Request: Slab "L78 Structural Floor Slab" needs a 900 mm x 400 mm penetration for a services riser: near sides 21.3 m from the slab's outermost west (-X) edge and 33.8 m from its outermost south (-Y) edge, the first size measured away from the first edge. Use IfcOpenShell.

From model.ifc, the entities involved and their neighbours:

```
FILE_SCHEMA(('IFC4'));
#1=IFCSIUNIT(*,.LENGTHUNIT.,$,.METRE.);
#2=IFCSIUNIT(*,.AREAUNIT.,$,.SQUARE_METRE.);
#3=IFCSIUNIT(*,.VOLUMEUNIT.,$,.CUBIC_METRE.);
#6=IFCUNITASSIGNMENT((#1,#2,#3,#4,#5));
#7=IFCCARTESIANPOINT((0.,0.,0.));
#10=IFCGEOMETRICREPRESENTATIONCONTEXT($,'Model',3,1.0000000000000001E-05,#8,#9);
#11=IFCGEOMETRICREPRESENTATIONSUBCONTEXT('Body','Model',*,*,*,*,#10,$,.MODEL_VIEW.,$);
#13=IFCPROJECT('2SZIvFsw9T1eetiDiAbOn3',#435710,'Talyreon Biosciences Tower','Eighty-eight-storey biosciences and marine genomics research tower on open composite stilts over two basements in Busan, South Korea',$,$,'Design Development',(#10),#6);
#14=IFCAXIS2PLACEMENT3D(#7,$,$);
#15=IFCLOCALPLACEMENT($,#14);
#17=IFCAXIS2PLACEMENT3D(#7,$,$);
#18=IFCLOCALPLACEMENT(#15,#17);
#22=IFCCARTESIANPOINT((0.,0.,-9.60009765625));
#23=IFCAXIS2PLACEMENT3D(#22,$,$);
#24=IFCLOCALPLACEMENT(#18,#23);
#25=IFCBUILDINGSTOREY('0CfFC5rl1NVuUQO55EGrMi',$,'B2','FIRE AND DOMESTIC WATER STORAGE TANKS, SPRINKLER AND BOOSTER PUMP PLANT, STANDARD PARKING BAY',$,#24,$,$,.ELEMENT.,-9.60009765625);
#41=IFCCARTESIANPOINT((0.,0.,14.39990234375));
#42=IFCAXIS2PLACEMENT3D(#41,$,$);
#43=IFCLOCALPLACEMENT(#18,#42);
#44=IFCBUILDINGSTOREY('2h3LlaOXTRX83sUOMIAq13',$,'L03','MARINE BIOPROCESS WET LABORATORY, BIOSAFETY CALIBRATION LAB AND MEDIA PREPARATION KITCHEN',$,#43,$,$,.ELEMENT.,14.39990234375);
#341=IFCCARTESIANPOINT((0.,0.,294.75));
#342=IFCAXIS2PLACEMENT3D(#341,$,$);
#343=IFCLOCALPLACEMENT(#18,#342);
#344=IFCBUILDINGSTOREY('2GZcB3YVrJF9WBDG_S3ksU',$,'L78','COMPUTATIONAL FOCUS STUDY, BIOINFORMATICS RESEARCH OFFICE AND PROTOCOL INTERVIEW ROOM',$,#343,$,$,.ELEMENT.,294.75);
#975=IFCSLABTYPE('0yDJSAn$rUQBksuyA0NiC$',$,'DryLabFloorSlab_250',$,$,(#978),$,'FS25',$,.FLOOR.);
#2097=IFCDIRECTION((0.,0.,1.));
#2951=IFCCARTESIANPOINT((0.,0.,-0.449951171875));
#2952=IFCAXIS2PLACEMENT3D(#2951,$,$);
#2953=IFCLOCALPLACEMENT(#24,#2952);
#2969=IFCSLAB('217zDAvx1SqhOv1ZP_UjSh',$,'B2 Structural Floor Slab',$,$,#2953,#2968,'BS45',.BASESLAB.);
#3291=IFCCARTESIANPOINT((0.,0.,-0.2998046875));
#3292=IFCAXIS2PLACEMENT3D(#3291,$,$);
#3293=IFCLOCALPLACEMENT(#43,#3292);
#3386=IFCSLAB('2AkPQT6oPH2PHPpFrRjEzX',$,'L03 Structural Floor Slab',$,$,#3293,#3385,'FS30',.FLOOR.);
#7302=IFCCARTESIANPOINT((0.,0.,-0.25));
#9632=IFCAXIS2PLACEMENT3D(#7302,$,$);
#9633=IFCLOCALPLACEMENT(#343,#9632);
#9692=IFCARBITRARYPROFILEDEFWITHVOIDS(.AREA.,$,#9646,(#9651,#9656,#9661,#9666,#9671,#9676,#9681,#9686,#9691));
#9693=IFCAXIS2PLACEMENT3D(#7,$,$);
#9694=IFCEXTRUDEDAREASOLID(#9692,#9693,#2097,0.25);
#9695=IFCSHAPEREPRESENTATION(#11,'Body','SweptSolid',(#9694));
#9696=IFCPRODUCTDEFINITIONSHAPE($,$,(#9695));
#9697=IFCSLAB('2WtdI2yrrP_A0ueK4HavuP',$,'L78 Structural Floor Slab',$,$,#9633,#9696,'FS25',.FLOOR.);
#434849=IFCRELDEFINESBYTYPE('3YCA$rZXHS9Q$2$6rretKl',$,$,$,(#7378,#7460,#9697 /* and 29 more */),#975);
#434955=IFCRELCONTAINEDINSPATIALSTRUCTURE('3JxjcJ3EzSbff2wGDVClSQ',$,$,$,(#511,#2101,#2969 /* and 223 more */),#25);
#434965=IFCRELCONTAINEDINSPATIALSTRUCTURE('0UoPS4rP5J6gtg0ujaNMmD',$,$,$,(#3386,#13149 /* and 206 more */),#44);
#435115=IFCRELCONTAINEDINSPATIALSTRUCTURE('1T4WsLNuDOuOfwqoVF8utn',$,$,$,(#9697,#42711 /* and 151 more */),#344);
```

```python
import numpy as np
import ifcopenshell
import ifcopenshell.api.feature
import ifcopenshell.api.geometry
import ifcopenshell.api.root
import ifcopenshell.geom
import ifcopenshell.util.placement
import ifcopenshell.util.representation
import ifcopenshell.util.shape
import ifcopenshell.util.unit

model = ifcopenshell.open("model.ifc")
unit_scale = ifcopenshell.util.unit.calculate_unit_scale(model)
settings = ifcopenshell.geom.settings()


def volume(element):
    """Net volume in cubic metres, openings subtracted."""
    shape = ifcopenshell.geom.create_shape(settings, element)
    return ifcopenshell.util.shape.get_volume(shape.geometry)


slab = model.by_guid("2WtdI2yrrP_A0ueK4HavuP")
before = volume(slab)

# Extent in the slab's own axes, in metres. The edges named are its -X and -Y sides.
slab_shape = ifcopenshell.geom.create_shape(settings, slab)
vertices = ifcopenshell.util.shape.get_vertices(slab_shape.geometry)
x_min, y_min, bottom = vertices.min(axis=0)
top = vertices[:, 2].max()

opening = ifcopenshell.api.root.create_entity(model, ifc_class="IfcOpeningElement", name="Services riser opening", predefined_type="OPENING")
context = ifcopenshell.util.representation.get_context(model, "Model", "Body", "MODEL_VIEW")
width, depth = 0.9, 0.4
outline = [(0.0, 0.0), (width, 0.0), (width, depth), (0.0, depth), (0.0, 0.0)]
# Overshoot both faces by 50 mm so the cut is clean.
shape = ifcopenshell.api.geometry.add_slab_representation(
    model, context=context, depth=top - bottom + 0.1, polyline=outline
)
ifcopenshell.api.geometry.assign_representation(model, product=opening, representation=shape)

matrix = ifcopenshell.util.placement.get_local_placement(slab.ObjectPlacement)
matrix[:, 3] = matrix @ np.append(np.array([x_min + 21.3, y_min + 33.8, bottom - 0.05]) / unit_scale, 1.0)
ifcopenshell.api.geometry.edit_object_placement(model, product=opening, matrix=matrix, is_si=False)
ifcopenshell.api.feature.add_feature(model, feature=opening, element=slab)

after = volume(slab)

print(f"slab volume {before:.3f} -> {after:.3f} m3")

model.write("model_updated.ifc")
```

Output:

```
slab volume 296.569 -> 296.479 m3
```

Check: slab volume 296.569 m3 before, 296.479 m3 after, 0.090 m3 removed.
